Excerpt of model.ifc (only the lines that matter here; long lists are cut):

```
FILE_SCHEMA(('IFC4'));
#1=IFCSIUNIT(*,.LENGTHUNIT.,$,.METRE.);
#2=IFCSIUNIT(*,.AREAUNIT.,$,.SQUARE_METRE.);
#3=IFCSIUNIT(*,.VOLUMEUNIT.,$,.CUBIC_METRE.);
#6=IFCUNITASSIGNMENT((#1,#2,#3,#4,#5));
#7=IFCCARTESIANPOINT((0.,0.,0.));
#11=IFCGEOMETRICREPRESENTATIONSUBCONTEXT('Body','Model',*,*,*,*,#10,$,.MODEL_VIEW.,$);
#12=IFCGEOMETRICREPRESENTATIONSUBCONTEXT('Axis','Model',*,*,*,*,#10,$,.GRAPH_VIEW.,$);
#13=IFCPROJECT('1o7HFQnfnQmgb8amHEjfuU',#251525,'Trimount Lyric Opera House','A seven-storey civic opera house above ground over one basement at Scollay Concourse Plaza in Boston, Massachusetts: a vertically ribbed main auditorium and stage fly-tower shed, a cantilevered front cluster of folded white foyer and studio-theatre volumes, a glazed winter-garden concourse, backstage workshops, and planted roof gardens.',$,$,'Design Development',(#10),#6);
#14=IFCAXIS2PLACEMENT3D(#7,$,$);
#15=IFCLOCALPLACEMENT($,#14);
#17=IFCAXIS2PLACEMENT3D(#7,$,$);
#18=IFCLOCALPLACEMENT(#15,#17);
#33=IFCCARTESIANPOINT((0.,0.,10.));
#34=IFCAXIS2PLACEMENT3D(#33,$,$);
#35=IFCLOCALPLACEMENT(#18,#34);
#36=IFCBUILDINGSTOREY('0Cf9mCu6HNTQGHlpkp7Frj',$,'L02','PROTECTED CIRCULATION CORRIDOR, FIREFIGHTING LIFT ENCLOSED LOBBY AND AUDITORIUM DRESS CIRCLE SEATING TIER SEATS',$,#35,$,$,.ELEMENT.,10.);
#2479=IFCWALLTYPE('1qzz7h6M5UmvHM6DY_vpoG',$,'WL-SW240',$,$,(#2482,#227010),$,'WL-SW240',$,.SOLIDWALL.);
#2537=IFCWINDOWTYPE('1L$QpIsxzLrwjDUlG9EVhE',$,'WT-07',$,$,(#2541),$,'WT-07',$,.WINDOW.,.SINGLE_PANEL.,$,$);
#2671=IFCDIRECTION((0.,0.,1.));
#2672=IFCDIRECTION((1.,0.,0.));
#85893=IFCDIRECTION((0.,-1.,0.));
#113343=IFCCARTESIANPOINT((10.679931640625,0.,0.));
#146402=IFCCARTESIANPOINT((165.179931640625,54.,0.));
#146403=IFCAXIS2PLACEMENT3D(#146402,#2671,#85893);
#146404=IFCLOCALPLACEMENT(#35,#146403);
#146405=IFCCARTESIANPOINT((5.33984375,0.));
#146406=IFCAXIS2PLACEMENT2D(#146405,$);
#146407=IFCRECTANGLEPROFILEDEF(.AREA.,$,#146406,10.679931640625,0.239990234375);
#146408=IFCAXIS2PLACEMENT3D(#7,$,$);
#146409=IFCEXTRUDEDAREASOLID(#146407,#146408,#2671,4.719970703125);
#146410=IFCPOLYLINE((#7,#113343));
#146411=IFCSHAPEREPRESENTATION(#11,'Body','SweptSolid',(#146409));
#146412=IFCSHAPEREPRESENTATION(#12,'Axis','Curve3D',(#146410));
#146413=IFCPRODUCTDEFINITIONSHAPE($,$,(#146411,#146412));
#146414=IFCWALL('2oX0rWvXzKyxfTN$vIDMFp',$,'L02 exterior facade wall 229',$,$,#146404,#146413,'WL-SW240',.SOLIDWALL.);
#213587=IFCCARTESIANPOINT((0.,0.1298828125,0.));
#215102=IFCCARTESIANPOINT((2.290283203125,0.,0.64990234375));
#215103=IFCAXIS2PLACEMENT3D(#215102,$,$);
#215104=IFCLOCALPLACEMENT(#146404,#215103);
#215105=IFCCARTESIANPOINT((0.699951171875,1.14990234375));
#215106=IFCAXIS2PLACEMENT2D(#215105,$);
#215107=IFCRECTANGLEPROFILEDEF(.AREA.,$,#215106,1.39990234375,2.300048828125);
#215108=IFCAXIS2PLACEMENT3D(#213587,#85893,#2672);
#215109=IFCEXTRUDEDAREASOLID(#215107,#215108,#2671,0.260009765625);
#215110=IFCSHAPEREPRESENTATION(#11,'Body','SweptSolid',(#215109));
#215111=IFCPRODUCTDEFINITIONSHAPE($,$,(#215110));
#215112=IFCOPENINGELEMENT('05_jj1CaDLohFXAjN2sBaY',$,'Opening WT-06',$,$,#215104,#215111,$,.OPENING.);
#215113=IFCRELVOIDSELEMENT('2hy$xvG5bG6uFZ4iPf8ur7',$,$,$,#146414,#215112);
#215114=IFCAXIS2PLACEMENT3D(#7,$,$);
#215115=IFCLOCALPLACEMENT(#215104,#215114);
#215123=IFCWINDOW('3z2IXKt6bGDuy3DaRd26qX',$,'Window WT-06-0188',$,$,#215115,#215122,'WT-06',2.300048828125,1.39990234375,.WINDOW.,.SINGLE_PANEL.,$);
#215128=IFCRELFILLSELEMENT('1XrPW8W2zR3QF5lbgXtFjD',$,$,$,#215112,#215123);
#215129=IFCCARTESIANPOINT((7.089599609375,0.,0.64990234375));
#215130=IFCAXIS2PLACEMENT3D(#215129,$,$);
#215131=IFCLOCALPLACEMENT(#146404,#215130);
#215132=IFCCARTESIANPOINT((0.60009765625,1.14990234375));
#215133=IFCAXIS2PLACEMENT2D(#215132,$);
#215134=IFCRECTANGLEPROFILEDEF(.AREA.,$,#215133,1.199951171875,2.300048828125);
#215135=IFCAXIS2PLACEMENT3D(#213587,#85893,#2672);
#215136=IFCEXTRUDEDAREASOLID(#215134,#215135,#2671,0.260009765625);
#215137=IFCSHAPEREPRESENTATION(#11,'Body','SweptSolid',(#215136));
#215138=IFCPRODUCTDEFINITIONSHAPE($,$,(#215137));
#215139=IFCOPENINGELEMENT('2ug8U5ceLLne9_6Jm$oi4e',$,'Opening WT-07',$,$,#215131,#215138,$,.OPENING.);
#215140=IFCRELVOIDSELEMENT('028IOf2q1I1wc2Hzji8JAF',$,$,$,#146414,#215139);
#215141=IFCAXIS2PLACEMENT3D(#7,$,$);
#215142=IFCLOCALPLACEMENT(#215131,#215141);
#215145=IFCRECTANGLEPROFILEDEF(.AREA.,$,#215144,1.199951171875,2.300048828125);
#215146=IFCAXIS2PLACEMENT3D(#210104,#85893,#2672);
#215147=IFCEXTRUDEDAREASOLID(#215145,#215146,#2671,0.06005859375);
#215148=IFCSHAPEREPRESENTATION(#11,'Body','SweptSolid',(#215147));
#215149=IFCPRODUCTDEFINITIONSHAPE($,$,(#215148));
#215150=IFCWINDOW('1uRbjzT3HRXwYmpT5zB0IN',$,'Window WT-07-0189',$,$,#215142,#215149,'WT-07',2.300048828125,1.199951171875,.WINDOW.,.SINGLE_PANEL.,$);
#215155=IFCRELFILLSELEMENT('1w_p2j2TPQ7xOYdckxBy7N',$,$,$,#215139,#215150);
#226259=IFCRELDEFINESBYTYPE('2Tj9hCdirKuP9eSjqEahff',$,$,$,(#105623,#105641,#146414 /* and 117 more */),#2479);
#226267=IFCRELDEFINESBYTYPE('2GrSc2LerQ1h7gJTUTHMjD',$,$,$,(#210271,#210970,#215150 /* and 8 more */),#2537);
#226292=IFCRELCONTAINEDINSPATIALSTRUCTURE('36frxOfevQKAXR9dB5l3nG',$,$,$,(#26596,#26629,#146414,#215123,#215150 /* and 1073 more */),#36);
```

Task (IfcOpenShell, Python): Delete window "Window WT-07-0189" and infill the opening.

```python
import ifcopenshell
import ifcopenshell.api.feature
import ifcopenshell.api.root
import ifcopenshell.geom
import ifcopenshell.util.shape

model = ifcopenshell.open("model.ifc")
settings = ifcopenshell.geom.settings()


def volume(element):
    """Net volume in cubic metres, openings subtracted."""
    shape = ifcopenshell.geom.create_shape(settings, element)
    return ifcopenshell.util.shape.get_volume(shape.geometry)


window = model.by_guid("1uRbjzT3HRXwYmpT5zB0IN")
opening = window.FillsVoids[0].RelatingOpeningElement
wall = opening.VoidsElements[0].RelatingBuildingElement
before = volume(wall)

ifcopenshell.api.root.remove_product(model, product=window)
ifcopenshell.api.feature.remove_feature(model, feature=opening)

after = volume(wall)

print(f"wall volume {before:.3f} -> {after:.3f} m3")

model.write("model_edited.ifc")
```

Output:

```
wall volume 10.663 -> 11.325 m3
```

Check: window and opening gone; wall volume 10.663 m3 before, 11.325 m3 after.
